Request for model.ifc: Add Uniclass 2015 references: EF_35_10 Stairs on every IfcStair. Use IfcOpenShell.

First a look at what the model holds.

```python
import ifcopenshell

model = ifcopenshell.open("model.ifc")
print(model.schema)
print("classifications:", [c.Name for c in model.by_type("IfcClassification")])
for ifc_class in ("IfcDoor", "IfcRoof", "IfcStair", "IfcWall", "IfcWindow"):
    print(ifc_class, len(model.by_type(ifc_class)))
```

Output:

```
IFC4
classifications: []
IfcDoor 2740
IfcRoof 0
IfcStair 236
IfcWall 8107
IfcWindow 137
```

```python
import ifcopenshell
import ifcopenshell.api.classification

model = ifcopenshell.open("model.ifc")

system = ifcopenshell.api.classification.add_classification(model, classification="Uniclass 2015")

codes = {
    "IfcStair": ("EF_35_10", "Stairs"),
}
for ifc_class, (code, name) in codes.items():
    products = model.by_type(ifc_class)
    ifcopenshell.api.classification.add_reference(
        model, products=products, classification=system, identification=code, name=name
    )
    print(code, len(products))

model.write("model_v2.ifc")
```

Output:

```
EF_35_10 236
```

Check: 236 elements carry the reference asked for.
